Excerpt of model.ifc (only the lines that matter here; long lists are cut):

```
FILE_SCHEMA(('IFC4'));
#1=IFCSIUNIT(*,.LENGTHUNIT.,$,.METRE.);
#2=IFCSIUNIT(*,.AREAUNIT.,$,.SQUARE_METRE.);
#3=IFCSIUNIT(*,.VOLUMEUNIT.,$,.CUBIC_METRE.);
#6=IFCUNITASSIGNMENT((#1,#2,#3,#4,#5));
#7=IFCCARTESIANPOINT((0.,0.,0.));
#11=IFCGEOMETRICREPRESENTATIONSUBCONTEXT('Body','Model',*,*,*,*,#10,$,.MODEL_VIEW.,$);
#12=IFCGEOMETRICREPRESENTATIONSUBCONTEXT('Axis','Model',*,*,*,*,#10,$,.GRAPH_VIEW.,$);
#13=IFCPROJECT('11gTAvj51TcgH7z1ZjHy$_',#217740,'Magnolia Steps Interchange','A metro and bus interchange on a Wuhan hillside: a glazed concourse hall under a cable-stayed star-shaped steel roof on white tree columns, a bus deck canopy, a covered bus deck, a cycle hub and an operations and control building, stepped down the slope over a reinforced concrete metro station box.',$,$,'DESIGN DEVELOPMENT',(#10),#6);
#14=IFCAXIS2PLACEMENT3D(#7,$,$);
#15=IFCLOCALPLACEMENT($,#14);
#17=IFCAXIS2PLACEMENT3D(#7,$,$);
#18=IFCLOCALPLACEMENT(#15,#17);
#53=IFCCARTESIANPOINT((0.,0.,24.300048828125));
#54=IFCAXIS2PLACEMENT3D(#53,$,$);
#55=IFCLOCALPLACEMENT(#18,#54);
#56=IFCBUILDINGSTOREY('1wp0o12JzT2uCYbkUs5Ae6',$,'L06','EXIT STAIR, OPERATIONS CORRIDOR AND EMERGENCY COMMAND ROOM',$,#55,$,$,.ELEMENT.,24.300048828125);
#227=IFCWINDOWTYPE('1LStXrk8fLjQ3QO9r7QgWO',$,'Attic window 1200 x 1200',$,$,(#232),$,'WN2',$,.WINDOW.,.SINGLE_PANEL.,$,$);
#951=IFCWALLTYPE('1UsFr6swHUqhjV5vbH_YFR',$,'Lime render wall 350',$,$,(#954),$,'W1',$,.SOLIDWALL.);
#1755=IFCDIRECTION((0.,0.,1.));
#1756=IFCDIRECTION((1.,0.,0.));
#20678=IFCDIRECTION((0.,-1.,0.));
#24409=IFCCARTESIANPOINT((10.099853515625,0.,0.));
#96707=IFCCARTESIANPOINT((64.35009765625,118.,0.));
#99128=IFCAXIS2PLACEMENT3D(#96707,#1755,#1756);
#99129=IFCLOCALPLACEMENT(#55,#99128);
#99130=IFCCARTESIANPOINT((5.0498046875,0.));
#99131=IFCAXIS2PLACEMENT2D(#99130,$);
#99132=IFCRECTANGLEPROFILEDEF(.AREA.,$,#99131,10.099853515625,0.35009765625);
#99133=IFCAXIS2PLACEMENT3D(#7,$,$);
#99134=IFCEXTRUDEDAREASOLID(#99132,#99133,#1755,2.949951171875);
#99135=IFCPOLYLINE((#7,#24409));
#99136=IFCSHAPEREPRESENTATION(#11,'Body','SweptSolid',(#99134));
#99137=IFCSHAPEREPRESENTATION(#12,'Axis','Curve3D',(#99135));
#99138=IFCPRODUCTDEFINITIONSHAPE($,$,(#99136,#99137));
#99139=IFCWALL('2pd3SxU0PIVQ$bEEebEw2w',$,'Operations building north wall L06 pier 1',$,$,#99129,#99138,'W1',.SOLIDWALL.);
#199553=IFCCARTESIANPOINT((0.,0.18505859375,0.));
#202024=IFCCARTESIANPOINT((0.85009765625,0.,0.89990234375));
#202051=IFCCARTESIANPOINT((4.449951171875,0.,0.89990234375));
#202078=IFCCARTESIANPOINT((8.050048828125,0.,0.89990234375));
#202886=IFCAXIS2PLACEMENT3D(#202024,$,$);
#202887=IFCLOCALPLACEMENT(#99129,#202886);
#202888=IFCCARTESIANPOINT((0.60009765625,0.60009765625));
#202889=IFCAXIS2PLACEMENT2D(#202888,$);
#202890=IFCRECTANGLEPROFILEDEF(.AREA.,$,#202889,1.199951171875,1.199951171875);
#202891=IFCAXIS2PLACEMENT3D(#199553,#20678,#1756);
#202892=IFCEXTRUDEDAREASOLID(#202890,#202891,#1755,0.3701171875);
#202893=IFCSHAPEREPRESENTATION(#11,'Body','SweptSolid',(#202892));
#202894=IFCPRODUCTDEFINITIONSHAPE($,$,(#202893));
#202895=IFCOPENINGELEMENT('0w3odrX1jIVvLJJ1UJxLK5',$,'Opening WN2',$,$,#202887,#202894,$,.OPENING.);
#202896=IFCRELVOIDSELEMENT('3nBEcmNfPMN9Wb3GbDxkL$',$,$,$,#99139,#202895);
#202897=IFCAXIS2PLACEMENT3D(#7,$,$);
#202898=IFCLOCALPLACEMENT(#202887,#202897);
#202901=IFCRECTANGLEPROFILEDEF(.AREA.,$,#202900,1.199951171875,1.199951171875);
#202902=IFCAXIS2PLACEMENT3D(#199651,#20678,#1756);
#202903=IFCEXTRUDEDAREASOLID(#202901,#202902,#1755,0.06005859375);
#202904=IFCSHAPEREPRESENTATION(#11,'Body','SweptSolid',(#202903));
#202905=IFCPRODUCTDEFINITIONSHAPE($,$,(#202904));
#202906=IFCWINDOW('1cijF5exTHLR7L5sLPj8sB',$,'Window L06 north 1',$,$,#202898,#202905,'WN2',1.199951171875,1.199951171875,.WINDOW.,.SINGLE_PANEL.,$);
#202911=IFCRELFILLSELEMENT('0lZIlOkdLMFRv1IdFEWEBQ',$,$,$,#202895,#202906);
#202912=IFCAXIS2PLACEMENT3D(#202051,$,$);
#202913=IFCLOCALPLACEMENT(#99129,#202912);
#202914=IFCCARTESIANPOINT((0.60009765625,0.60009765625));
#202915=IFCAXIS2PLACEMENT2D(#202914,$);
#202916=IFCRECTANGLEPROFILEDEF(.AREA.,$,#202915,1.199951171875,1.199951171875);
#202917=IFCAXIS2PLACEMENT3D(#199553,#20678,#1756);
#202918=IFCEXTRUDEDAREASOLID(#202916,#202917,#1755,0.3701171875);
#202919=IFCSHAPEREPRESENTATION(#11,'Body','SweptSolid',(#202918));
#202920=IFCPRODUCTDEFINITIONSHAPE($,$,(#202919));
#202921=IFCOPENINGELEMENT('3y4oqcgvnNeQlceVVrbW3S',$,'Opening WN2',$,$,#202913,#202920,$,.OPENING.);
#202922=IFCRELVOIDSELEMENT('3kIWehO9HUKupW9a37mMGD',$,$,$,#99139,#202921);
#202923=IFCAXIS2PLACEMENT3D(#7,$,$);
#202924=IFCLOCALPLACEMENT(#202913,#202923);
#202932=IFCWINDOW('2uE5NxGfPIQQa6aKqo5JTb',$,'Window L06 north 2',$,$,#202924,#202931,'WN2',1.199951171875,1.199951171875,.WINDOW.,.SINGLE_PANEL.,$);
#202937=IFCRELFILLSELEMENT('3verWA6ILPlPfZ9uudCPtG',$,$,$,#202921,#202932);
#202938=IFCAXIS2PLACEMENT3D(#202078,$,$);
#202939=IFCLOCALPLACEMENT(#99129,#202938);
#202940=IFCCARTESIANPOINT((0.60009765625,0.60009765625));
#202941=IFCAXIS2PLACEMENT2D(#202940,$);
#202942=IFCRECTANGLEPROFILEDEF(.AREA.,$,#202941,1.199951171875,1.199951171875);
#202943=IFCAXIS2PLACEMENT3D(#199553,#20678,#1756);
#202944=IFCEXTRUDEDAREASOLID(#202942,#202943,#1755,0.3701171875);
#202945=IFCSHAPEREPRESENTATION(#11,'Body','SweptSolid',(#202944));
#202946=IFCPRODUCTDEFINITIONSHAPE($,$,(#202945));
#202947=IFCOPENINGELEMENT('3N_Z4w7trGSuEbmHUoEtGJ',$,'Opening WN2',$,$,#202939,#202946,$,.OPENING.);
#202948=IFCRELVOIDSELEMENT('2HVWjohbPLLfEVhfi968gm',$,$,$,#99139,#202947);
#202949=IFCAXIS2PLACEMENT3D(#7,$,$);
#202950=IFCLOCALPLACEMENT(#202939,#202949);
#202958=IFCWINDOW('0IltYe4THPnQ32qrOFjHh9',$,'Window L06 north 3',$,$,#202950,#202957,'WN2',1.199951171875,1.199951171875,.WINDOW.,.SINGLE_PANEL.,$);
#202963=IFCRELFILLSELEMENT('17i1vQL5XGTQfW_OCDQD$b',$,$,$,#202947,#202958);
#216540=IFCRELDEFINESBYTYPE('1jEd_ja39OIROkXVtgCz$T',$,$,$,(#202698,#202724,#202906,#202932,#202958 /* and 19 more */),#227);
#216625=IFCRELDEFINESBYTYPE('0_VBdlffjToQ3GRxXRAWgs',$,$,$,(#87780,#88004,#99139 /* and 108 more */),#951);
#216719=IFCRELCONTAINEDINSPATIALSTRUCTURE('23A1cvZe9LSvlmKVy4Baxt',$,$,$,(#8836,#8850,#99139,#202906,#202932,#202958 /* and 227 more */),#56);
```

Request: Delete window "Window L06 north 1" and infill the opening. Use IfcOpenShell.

```python
import ifcopenshell
import ifcopenshell.api.feature
import ifcopenshell.api.root
import ifcopenshell.geom
import ifcopenshell.util.shape

model = ifcopenshell.open("model.ifc")
settings = ifcopenshell.geom.settings()


def volume(element):
    """Net volume in cubic metres, openings subtracted."""
    shape = ifcopenshell.geom.create_shape(settings, element)
    return ifcopenshell.util.shape.get_volume(shape.geometry)


window = model.by_guid("1cijF5exTHLR7L5sLPj8sB")
opening = window.FillsVoids[0].RelatingOpeningElement
wall = opening.VoidsElements[0].RelatingBuildingElement
before = volume(wall)

ifcopenshell.api.root.remove_product(model, product=window)
ifcopenshell.api.feature.remove_feature(model, feature=opening)

after = volume(wall)

print(f"wall volume {before:.3f} -> {after:.3f} m3")

model.write("model-out.ifc")
```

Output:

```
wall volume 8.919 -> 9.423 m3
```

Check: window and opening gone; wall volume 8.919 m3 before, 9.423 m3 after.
